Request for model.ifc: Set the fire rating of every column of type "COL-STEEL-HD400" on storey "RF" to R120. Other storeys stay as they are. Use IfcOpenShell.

First a look at what the model holds.

```python
import ifcopenshell
import ifcopenshell.util.element

model = ifcopenshell.open("model.ifc")
print(model.schema)
storey = next(s for s in model.by_type("IfcBuildingStorey") if s.Name == "RF")
columns = [e for e in ifcopenshell.util.element.get_decomposition(storey) if e.is_a("IfcColumn")]
seen = {}
for e in columns:
    element_type = ifcopenshell.util.element.get_type(e)
    key = (element_type.Name if element_type != e and element_type else None, ifcopenshell.util.element.get_pset(e, "Pset_ColumnCommon", "FireRating"))
    seen[key] = seen.get(key, 0) + 1
for (name, value), count in sorted(seen.items(), key=str):
    print(count, "x", name, "|", value)
```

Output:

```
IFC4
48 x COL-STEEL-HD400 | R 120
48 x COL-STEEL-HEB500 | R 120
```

```python
import ifcopenshell
import ifcopenshell.api.pset
import ifcopenshell.util.element

model = ifcopenshell.open("model.ifc")

storey = next(s for s in model.by_type("IfcBuildingStorey") if s.Name == "RF")
columns = [e for e in ifcopenshell.util.element.get_decomposition(storey) if e.is_a("IfcColumn")]

count = 0
for e in columns:
    element_type = ifcopenshell.util.element.get_type(e)
    if element_type in (None, e) or element_type.Name != "COL-STEEL-HD400":
        continue
    # add_pset returns the element's existing set when there is one.
    pset = ifcopenshell.api.pset.add_pset(model, product=e, name="Pset_ColumnCommon")
    ifcopenshell.api.pset.edit_pset(model, pset=pset, properties={"FireRating": "R120"})
    count += 1

print(count, "columns updated")

model.write("model_edited.ifc")
```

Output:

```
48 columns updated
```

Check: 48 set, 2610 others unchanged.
